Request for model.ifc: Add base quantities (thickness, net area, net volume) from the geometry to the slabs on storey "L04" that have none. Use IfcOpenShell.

First a look at what the model holds.

```python
import ifcopenshell
import ifcopenshell.util.element
import ifcopenshell.util.unit

model = ifcopenshell.open("model.ifc")
print(model.schema)
for unit_type in ("LENGTHUNIT", "AREAUNIT", "VOLUMEUNIT"):
    print(unit_type, ifcopenshell.util.unit.calculate_unit_scale(model, unit_type))
storey = next(s for s in model.by_type("IfcBuildingStorey") if s.Name == "L04")
slabs = [e for e in ifcopenshell.util.element.get_decomposition(storey) if e.is_a("IfcSlab")]
for e in sorted(slabs, key=lambda e: e.id()):
    print(e.id(), e.is_a(), e.Name, list(ifcopenshell.util.element.get_psets(e, qtos_only=True)), sep=" | ")
```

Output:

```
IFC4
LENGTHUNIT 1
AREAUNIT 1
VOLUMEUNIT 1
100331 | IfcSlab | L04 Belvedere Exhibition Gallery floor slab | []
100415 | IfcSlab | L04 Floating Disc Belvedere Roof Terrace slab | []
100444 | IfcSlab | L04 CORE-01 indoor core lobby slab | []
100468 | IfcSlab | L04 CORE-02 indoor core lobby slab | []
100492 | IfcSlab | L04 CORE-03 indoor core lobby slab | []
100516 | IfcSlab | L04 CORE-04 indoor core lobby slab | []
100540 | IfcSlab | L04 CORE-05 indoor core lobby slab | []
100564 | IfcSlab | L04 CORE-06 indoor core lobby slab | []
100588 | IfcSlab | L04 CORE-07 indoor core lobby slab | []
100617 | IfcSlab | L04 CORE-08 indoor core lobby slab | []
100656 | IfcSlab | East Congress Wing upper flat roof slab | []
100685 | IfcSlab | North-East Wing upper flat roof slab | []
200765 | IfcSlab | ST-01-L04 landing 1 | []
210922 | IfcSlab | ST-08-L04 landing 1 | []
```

```python
import ifcopenshell
import ifcopenshell.api.pset
import ifcopenshell.geom
import ifcopenshell.util.element
import ifcopenshell.util.shape
import ifcopenshell.util.unit

model = ifcopenshell.open("model.ifc")
unit_scale = ifcopenshell.util.unit.calculate_unit_scale(model)
area_scale = ifcopenshell.util.unit.calculate_unit_scale(model, "AREAUNIT")
volume_scale = ifcopenshell.util.unit.calculate_unit_scale(model, "VOLUMEUNIT")
settings = ifcopenshell.geom.settings()

storey = next(s for s in model.by_type("IfcBuildingStorey") if s.Name == "L04")
slabs = [e for e in ifcopenshell.util.element.get_decomposition(storey) if e.is_a("IfcSlab")]

for e in sorted(slabs, key=lambda e: e.id()):
    if ifcopenshell.util.element.get_psets(e, qtos_only=True, should_inherit=False):
        continue
    # Geometry comes back in metres, in the element's own axes.
    shape = ifcopenshell.geom.create_shape(settings, e)
    values = {
        "Width": ifcopenshell.util.shape.get_z(shape.geometry) / unit_scale,
        "NetArea": ifcopenshell.util.shape.get_footprint_area(shape.geometry) / area_scale,
        "NetVolume": ifcopenshell.util.shape.get_volume(shape.geometry) / volume_scale,
    }
    qto = ifcopenshell.api.pset.add_qto(model, product=e, name="Qto_SlabBaseQuantities")
    ifcopenshell.api.pset.edit_qto(model, qto=qto, properties=values)
    print(e.id(), {k: round(v, 3) for k, v in values.items()})

model.write("model_rev.ifc")
```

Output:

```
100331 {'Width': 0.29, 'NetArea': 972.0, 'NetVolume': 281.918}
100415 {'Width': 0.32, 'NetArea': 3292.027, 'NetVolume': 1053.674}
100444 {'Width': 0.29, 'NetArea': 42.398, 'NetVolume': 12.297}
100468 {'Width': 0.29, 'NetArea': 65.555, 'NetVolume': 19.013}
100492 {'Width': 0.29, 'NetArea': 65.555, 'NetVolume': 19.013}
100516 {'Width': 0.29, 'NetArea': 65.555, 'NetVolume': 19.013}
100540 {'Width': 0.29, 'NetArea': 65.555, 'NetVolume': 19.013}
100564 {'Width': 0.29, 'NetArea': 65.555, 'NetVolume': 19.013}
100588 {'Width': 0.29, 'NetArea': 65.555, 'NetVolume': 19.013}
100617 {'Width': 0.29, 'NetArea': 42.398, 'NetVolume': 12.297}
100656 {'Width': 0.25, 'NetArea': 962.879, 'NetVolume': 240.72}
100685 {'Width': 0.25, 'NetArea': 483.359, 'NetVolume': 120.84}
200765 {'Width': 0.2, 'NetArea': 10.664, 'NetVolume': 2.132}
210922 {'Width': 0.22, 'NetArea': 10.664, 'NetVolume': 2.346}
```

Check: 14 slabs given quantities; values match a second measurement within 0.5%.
